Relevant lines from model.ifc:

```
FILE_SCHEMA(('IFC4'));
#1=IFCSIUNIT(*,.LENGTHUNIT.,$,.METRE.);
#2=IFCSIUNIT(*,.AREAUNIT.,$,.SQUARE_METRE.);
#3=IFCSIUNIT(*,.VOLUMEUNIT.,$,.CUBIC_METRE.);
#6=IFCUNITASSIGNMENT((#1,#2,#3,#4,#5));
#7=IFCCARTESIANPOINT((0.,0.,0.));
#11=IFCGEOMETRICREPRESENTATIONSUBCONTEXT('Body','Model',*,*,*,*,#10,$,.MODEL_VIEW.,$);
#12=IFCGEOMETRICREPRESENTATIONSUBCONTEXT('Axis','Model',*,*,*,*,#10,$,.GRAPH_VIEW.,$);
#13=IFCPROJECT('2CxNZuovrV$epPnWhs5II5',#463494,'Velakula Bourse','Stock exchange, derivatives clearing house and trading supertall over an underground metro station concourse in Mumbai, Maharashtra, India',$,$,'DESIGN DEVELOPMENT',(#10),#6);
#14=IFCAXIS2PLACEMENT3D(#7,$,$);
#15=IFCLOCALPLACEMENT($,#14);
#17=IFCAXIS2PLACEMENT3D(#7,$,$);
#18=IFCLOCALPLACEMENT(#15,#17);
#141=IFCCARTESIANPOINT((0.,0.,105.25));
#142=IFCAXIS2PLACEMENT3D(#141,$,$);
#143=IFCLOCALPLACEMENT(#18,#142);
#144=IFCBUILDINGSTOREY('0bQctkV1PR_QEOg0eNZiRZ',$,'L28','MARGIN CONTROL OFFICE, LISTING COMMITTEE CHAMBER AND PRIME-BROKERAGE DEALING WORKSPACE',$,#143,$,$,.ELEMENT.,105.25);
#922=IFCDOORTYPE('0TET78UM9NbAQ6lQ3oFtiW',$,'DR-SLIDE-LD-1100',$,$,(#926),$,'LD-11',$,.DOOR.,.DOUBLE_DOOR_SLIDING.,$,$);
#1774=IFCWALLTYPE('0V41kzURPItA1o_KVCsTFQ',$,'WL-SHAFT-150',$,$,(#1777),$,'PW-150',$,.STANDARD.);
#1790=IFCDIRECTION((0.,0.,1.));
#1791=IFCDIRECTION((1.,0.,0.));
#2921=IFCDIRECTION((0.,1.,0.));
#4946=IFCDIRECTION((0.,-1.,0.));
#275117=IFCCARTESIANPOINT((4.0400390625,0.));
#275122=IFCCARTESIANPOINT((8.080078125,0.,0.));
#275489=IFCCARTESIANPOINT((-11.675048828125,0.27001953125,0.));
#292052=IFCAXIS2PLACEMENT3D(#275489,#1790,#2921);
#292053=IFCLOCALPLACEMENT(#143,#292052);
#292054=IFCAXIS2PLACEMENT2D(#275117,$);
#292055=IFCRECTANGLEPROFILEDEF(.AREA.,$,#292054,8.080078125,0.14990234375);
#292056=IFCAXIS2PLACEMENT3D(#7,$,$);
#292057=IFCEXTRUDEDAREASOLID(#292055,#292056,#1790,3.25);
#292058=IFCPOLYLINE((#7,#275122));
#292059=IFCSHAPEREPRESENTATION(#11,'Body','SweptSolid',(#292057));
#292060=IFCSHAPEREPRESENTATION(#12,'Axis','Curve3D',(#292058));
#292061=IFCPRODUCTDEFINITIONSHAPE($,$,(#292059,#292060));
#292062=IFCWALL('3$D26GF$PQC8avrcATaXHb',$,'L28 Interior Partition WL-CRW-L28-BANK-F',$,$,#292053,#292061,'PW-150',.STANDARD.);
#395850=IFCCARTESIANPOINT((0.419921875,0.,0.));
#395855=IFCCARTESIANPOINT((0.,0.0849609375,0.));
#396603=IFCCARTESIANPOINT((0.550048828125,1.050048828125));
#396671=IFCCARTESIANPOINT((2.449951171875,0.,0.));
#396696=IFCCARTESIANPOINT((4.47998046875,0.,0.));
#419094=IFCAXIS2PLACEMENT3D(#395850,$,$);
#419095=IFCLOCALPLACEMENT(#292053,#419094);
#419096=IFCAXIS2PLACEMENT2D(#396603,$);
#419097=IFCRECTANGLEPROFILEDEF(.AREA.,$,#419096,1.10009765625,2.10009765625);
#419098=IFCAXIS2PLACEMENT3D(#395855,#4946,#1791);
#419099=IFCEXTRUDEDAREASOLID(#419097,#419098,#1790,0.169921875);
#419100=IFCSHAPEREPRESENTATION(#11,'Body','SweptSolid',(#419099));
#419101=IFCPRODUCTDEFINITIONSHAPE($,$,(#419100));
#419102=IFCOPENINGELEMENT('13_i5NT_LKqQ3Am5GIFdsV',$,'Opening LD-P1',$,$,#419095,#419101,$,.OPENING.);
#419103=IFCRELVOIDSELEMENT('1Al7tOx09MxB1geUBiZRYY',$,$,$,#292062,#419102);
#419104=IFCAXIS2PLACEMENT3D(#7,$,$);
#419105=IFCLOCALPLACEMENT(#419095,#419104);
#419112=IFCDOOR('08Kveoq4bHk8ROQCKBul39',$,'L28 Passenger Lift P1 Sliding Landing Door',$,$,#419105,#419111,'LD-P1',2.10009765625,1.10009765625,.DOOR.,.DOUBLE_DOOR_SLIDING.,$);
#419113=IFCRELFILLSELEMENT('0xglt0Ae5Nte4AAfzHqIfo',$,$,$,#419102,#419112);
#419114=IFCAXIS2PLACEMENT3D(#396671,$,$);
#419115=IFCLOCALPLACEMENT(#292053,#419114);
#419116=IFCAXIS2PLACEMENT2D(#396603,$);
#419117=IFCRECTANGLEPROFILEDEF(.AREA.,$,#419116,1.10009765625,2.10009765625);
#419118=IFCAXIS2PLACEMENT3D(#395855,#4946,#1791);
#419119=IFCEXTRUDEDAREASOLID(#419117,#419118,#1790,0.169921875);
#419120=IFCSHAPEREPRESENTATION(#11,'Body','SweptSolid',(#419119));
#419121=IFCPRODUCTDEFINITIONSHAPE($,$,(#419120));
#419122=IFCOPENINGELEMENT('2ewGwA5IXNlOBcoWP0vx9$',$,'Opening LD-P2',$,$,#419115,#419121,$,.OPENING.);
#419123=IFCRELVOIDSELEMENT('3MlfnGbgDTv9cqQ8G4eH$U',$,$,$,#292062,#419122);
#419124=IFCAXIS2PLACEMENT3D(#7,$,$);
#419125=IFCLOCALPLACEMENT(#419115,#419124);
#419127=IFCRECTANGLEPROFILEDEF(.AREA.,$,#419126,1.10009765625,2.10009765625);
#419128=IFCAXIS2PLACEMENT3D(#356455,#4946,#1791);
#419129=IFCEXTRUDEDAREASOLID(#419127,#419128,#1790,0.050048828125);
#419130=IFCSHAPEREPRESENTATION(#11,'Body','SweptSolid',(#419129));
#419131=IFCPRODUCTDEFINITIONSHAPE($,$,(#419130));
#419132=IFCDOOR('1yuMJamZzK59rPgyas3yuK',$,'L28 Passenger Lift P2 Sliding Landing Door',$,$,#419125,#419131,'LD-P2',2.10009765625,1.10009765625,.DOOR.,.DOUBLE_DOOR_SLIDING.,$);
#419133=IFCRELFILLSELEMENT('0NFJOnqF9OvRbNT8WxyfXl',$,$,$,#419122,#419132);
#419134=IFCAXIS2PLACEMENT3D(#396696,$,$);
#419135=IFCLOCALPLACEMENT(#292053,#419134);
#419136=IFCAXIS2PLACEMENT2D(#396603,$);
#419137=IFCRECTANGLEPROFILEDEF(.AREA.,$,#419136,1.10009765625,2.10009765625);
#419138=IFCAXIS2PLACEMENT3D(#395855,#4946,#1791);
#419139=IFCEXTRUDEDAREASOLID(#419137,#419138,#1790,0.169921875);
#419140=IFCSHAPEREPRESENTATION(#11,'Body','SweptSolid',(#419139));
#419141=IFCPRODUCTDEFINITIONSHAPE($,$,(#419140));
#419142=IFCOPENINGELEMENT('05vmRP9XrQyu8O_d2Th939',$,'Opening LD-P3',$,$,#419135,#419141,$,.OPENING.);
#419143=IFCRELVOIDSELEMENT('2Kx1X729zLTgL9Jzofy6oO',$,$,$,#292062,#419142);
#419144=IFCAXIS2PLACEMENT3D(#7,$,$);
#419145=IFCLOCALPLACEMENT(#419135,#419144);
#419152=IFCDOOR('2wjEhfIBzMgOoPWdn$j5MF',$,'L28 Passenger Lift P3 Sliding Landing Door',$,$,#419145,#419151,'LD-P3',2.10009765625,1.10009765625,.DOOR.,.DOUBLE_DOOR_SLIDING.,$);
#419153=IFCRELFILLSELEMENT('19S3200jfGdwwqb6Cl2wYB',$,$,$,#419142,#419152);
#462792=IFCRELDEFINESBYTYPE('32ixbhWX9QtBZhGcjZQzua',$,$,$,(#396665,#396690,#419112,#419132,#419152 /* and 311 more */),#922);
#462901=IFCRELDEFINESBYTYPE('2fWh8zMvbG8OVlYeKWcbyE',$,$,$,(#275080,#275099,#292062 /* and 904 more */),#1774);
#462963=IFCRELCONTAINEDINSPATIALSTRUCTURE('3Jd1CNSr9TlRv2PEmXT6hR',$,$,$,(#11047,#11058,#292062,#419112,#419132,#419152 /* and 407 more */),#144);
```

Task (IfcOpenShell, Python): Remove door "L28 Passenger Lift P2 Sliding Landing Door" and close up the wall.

```python
import ifcopenshell
import ifcopenshell.api.feature
import ifcopenshell.api.root
import ifcopenshell.geom
import ifcopenshell.util.shape

model = ifcopenshell.open("model.ifc")
settings = ifcopenshell.geom.settings()


def volume(element):
    """Net volume in cubic metres, openings subtracted."""
    shape = ifcopenshell.geom.create_shape(settings, element)
    return ifcopenshell.util.shape.get_volume(shape.geometry)


door = model.by_id(419132)
opening = door.FillsVoids[0].RelatingOpeningElement
wall = opening.VoidsElements[0].RelatingBuildingElement
before = volume(wall)

ifcopenshell.api.root.remove_product(model, product=door)
ifcopenshell.api.feature.remove_feature(model, feature=opening)

after = volume(wall)

print(f"wall volume {before:.3f} -> {after:.3f} m3")

model.write("model_updated.ifc")
```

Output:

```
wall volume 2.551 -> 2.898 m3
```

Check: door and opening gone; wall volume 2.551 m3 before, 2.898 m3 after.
